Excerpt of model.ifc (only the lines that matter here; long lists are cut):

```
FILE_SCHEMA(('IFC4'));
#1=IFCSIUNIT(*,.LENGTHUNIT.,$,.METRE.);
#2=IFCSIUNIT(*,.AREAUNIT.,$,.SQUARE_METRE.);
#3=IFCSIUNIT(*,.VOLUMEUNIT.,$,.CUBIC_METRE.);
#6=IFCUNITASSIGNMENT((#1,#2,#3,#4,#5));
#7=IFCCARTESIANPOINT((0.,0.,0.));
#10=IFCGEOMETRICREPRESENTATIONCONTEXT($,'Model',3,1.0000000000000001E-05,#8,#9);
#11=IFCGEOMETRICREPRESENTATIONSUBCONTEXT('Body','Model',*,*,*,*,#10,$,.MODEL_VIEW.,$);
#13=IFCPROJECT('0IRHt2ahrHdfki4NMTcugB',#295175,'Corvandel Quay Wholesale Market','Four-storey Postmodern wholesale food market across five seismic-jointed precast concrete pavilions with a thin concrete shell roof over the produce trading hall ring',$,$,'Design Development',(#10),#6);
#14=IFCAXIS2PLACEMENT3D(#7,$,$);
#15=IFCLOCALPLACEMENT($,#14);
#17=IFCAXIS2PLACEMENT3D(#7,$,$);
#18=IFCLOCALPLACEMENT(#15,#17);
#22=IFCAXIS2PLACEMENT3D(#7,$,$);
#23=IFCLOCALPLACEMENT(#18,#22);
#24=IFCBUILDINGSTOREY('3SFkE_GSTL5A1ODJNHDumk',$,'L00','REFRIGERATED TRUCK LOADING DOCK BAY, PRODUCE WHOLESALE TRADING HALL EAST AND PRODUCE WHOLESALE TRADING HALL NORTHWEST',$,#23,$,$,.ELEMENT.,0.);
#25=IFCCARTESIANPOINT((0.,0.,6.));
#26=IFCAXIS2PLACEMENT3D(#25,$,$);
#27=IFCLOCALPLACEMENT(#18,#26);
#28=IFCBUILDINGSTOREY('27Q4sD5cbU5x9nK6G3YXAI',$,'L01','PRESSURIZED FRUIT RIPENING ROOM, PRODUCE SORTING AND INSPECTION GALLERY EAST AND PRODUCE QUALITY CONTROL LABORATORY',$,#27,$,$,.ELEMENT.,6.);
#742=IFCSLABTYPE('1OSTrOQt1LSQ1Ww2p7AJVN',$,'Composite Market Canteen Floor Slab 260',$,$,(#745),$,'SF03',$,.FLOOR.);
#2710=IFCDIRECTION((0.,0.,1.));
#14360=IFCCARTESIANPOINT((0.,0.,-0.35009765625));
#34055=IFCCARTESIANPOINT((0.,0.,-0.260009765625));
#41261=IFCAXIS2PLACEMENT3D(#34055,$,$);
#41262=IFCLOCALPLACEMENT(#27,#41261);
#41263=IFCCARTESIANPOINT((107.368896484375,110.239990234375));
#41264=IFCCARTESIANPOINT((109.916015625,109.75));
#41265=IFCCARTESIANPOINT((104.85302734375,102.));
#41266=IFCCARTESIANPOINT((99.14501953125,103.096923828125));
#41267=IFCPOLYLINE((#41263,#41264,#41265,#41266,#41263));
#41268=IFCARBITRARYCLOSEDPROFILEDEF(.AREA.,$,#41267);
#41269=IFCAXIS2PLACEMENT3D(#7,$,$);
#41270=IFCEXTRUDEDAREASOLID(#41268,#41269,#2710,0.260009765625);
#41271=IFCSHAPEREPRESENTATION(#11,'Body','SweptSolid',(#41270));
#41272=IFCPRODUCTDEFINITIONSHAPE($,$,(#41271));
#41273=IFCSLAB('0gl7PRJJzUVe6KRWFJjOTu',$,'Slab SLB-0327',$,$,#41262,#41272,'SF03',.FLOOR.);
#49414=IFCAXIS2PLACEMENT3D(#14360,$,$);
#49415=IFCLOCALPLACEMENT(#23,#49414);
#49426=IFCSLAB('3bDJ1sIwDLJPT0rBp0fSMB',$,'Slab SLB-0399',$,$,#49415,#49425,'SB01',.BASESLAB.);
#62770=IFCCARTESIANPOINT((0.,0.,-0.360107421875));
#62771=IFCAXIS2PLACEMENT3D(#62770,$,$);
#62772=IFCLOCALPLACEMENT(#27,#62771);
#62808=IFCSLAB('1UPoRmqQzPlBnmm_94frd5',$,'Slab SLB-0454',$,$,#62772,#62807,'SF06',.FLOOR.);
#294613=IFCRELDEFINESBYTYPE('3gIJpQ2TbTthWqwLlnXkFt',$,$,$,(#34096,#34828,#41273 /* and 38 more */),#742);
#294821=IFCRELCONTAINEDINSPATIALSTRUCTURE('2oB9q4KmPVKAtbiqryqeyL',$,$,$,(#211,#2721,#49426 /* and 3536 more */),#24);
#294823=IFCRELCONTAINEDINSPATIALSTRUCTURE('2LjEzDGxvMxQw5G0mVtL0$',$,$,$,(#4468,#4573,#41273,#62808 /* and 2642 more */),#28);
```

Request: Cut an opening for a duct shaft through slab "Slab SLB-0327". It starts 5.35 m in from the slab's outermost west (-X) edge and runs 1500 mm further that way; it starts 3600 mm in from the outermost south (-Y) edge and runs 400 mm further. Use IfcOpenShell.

```python
import numpy as np
import ifcopenshell
import ifcopenshell.api.feature
import ifcopenshell.api.geometry
import ifcopenshell.api.root
import ifcopenshell.geom
import ifcopenshell.util.placement
import ifcopenshell.util.representation
import ifcopenshell.util.shape
import ifcopenshell.util.unit

model = ifcopenshell.open("model.ifc")
unit_scale = ifcopenshell.util.unit.calculate_unit_scale(model)
settings = ifcopenshell.geom.settings()


def volume(element):
    """Net volume in cubic metres, openings subtracted."""
    shape = ifcopenshell.geom.create_shape(settings, element)
    return ifcopenshell.util.shape.get_volume(shape.geometry)


slab = model.by_id(41273)
before = volume(slab)

# Extent in the slab's own axes, in metres. The edges named are its -X and -Y sides.
slab_shape = ifcopenshell.geom.create_shape(settings, slab)
vertices = ifcopenshell.util.shape.get_vertices(slab_shape.geometry)
x_min, y_min, bottom = vertices.min(axis=0)
top = vertices[:, 2].max()

opening = ifcopenshell.api.root.create_entity(model, ifc_class="IfcOpeningElement", name="Duct shaft opening", predefined_type="OPENING")
context = ifcopenshell.util.representation.get_context(model, "Model", "Body", "MODEL_VIEW")
width, depth = 1.5, 0.4
outline = [(0.0, 0.0), (width, 0.0), (width, depth), (0.0, depth), (0.0, 0.0)]
# Overshoot both faces by 50 mm so the cut is clean.
shape = ifcopenshell.api.geometry.add_slab_representation(
    model, context=context, depth=top - bottom + 0.1, polyline=outline
)
ifcopenshell.api.geometry.assign_representation(model, product=opening, representation=shape)

matrix = ifcopenshell.util.placement.get_local_placement(slab.ObjectPlacement)
matrix[:, 3] = matrix @ np.append(np.array([x_min + 5.35, y_min + 3.6, bottom - 0.05]) / unit_scale, 1.0)
ifcopenshell.api.geometry.edit_object_placement(model, product=opening, matrix=matrix, is_si=False)
ifcopenshell.api.feature.add_feature(model, feature=opening, element=slab)

after = volume(slab)

print(f"slab volume {before:.3f} -> {after:.3f} m3")

model.write("model_edited.ifc")
```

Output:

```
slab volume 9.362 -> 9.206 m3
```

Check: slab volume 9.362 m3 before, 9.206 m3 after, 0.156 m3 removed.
